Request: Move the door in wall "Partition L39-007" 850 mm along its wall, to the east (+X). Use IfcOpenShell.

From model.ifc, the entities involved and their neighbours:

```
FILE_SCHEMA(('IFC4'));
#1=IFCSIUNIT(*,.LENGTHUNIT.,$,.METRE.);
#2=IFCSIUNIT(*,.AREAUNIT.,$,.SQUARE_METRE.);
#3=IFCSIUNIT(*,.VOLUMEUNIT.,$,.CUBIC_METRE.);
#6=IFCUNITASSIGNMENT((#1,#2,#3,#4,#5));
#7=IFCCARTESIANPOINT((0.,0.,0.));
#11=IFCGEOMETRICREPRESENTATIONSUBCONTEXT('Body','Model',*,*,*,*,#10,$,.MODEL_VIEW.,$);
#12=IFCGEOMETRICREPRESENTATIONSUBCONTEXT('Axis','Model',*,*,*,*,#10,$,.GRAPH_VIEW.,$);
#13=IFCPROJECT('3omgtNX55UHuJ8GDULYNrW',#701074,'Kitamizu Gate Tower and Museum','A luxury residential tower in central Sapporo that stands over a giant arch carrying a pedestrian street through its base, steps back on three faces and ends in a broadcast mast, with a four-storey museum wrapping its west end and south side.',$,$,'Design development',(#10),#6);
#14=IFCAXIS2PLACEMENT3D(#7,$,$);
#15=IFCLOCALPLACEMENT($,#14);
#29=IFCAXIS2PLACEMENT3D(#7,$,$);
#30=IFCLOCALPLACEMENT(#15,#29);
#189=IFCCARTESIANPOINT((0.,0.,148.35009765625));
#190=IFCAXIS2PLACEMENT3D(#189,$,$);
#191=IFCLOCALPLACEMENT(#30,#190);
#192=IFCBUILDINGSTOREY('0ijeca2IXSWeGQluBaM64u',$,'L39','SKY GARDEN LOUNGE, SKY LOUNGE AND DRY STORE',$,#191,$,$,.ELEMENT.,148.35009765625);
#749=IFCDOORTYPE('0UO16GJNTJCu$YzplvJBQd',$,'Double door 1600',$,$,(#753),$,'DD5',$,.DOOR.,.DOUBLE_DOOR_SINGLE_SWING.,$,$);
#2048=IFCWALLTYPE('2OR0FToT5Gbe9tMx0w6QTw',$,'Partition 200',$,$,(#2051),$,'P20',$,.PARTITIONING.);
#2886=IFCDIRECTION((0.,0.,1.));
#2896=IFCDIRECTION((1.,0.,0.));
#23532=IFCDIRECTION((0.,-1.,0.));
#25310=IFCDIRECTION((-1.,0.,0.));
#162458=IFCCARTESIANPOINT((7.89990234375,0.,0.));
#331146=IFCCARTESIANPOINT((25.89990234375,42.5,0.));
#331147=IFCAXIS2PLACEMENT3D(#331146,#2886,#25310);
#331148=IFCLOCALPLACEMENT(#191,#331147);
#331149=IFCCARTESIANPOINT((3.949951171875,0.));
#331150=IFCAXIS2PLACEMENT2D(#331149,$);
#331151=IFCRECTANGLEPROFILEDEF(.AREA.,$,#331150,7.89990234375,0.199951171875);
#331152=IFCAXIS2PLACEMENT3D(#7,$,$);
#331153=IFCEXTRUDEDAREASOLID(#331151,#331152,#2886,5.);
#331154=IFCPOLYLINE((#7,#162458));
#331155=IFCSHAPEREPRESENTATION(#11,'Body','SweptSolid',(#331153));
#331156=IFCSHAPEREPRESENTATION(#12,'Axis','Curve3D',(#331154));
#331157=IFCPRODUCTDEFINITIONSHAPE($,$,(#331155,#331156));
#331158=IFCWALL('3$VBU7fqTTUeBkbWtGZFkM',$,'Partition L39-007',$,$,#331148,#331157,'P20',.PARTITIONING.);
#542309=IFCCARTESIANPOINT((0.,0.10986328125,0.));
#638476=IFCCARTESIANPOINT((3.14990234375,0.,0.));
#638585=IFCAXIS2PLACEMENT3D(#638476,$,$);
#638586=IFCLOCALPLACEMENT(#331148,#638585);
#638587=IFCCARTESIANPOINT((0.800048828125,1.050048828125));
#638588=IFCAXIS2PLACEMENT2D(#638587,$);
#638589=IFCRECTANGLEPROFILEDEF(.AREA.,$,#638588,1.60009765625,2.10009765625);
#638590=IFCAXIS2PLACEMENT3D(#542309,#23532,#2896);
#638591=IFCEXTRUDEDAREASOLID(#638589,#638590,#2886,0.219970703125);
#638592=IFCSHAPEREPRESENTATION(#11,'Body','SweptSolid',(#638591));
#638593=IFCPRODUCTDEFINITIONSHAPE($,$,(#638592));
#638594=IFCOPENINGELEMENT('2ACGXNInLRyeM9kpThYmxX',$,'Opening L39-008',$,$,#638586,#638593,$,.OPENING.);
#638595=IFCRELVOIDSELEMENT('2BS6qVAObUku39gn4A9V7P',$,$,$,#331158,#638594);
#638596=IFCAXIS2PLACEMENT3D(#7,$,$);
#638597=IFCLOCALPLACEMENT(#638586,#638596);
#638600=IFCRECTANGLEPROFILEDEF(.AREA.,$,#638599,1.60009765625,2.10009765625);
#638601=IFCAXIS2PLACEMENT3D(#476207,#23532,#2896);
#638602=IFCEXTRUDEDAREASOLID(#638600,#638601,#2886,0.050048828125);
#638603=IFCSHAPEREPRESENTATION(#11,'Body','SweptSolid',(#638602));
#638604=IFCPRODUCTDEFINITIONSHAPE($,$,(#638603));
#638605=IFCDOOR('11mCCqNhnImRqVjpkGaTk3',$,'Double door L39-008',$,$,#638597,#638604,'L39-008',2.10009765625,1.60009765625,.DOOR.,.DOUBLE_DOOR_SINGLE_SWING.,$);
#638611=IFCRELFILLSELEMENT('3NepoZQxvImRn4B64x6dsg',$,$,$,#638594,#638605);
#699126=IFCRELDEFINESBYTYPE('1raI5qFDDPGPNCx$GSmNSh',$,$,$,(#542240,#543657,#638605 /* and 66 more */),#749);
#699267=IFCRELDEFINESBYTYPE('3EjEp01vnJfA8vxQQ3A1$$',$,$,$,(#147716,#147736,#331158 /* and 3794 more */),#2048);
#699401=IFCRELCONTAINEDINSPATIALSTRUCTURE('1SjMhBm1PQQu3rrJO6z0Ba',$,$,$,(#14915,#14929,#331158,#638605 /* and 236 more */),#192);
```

```python
import ifcopenshell
import ifcopenshell.api.geometry
import ifcopenshell.util.placement

model = ifcopenshell.open("model.ifc")

door = model.by_id(638605)
opening = door.FillsVoids[0].RelatingOpeningElement
wall = opening.VoidsElements[0].RelatingBuildingElement

wall_matrix = ifcopenshell.util.placement.get_local_placement(wall.ObjectPlacement)
shift = wall_matrix[:3, 0] * -0.85
before = ifcopenshell.util.placement.get_local_placement(door.ObjectPlacement)[:3, 3].copy()

# The door is placed relative to its opening, so it follows when the opening moves.
matrix = ifcopenshell.util.placement.get_local_placement(opening.ObjectPlacement)
matrix[:3, 3] += shift
ifcopenshell.api.geometry.edit_object_placement(
    model, product=opening, matrix=matrix, is_si=False, should_transform_children=True
)

after = ifcopenshell.util.placement.get_local_placement(door.ObjectPlacement)[:3, 3]
print("door moved by", (after - before).round(3) + 0.0)

model.write("model_v2.ifc")
```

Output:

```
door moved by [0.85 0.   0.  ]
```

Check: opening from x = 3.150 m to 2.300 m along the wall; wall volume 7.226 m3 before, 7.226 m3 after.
